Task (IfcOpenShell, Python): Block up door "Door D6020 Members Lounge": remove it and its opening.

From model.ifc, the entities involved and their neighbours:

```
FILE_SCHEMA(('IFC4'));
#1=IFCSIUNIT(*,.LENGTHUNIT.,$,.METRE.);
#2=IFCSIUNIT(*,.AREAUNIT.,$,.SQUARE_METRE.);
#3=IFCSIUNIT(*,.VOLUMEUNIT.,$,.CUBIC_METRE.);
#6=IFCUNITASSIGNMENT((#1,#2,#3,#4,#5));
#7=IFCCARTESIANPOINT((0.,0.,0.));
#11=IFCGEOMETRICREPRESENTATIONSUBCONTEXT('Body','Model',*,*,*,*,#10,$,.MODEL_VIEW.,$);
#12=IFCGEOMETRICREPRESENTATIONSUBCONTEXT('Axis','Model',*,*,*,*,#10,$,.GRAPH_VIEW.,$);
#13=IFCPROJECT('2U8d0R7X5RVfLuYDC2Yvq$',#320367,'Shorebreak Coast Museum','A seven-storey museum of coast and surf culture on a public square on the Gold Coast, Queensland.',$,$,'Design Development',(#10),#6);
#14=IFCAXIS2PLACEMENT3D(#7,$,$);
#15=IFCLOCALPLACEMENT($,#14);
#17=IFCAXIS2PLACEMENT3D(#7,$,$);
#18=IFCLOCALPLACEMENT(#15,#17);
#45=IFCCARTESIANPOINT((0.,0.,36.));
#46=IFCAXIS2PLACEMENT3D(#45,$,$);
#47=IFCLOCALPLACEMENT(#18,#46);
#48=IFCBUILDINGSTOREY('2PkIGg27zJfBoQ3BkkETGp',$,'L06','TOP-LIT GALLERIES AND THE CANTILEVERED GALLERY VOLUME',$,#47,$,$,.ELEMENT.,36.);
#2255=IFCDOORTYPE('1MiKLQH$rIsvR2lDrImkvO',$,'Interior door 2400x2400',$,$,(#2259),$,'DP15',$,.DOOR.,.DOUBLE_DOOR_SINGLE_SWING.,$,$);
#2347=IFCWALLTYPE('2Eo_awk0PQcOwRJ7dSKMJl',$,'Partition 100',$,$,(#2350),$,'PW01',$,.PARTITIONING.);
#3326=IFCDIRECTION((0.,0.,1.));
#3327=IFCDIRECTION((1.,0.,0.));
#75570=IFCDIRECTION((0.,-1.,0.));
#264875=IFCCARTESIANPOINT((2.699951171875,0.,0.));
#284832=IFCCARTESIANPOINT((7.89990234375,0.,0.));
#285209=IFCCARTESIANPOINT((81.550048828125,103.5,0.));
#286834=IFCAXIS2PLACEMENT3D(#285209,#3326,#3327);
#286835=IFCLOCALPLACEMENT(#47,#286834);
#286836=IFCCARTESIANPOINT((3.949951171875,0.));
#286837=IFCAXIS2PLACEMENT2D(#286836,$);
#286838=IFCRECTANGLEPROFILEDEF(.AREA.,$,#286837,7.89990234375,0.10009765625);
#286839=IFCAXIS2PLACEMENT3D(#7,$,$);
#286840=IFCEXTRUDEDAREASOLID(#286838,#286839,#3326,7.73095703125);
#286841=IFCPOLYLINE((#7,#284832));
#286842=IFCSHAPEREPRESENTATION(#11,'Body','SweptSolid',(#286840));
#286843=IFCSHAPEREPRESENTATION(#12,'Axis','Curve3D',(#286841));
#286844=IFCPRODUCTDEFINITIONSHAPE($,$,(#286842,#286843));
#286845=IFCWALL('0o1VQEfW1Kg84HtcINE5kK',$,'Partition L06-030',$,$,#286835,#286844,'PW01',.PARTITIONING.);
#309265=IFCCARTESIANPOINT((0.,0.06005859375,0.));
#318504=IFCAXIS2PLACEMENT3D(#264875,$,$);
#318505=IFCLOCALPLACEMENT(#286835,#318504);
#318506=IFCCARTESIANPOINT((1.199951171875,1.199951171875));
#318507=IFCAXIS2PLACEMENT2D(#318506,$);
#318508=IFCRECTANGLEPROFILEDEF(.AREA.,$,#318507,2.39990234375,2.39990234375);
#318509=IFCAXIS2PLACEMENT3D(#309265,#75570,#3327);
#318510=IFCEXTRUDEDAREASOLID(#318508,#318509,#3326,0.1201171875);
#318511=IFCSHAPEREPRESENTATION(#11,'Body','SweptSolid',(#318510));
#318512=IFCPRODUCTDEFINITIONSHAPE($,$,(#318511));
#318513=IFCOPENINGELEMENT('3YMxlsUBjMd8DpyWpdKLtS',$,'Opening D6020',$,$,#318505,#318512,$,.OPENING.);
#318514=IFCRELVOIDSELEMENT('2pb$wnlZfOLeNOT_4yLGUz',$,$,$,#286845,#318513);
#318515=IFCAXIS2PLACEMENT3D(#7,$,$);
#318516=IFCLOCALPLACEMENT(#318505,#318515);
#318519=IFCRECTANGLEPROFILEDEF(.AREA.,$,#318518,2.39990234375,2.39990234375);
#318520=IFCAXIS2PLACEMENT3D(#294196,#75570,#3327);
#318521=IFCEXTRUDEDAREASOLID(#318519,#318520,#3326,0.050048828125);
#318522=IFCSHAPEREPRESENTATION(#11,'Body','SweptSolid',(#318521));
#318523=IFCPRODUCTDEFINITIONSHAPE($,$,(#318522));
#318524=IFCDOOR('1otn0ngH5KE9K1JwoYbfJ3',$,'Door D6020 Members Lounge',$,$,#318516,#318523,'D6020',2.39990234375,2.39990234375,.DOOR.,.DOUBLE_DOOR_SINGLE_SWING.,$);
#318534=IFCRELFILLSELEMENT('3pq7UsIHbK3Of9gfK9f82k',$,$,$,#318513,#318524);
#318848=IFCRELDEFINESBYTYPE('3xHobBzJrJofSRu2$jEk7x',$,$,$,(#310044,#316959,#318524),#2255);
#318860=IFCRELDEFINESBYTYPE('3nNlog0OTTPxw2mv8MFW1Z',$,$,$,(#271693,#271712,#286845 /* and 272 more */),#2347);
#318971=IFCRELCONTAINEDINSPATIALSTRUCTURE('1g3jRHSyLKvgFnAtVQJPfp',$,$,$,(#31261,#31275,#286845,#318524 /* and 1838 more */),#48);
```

```python
import ifcopenshell
import ifcopenshell.api.feature
import ifcopenshell.api.root
import ifcopenshell.geom
import ifcopenshell.util.shape

model = ifcopenshell.open("model.ifc")
settings = ifcopenshell.geom.settings()


def volume(element):
    """Net volume in cubic metres, openings subtracted."""
    shape = ifcopenshell.geom.create_shape(settings, element)
    return ifcopenshell.util.shape.get_volume(shape.geometry)


door = model.by_guid("1otn0ngH5KE9K1JwoYbfJ3")
opening = door.FillsVoids[0].RelatingOpeningElement
wall = opening.VoidsElements[0].RelatingBuildingElement
before = volume(wall)

ifcopenshell.api.root.remove_product(model, product=door)
ifcopenshell.api.feature.remove_feature(model, feature=opening)

after = volume(wall)

print(f"wall volume {before:.3f} -> {after:.3f} m3")

model.write("model_updated.ifc")
```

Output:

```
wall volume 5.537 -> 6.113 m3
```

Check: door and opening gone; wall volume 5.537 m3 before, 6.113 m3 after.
